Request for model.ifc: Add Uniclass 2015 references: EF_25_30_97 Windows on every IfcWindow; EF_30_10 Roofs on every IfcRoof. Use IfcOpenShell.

First a look at what the model holds.

```python
import ifcopenshell

model = ifcopenshell.open("model.ifc")
print(model.schema)
print("classifications:", [c.Name for c in model.by_type("IfcClassification")])
for ifc_class in ("IfcDoor", "IfcRoof", "IfcStair", "IfcWall", "IfcWindow"):
    print(ifc_class, len(model.by_type(ifc_class)))
```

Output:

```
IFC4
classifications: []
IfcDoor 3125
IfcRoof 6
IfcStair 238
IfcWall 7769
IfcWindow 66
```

```python
import ifcopenshell
import ifcopenshell.api.classification

model = ifcopenshell.open("model.ifc")

system = ifcopenshell.api.classification.add_classification(model, classification="Uniclass 2015")

codes = {
    "IfcWindow": ("EF_25_30_97", "Windows"),
    "IfcRoof": ("EF_30_10", "Roofs"),
}
for ifc_class, (code, name) in codes.items():
    products = model.by_type(ifc_class)
    ifcopenshell.api.classification.add_reference(
        model, products=products, classification=system, identification=code, name=name
    )
    print(code, len(products))

model.write("model_rev.ifc")
```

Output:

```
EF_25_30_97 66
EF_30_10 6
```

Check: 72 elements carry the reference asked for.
